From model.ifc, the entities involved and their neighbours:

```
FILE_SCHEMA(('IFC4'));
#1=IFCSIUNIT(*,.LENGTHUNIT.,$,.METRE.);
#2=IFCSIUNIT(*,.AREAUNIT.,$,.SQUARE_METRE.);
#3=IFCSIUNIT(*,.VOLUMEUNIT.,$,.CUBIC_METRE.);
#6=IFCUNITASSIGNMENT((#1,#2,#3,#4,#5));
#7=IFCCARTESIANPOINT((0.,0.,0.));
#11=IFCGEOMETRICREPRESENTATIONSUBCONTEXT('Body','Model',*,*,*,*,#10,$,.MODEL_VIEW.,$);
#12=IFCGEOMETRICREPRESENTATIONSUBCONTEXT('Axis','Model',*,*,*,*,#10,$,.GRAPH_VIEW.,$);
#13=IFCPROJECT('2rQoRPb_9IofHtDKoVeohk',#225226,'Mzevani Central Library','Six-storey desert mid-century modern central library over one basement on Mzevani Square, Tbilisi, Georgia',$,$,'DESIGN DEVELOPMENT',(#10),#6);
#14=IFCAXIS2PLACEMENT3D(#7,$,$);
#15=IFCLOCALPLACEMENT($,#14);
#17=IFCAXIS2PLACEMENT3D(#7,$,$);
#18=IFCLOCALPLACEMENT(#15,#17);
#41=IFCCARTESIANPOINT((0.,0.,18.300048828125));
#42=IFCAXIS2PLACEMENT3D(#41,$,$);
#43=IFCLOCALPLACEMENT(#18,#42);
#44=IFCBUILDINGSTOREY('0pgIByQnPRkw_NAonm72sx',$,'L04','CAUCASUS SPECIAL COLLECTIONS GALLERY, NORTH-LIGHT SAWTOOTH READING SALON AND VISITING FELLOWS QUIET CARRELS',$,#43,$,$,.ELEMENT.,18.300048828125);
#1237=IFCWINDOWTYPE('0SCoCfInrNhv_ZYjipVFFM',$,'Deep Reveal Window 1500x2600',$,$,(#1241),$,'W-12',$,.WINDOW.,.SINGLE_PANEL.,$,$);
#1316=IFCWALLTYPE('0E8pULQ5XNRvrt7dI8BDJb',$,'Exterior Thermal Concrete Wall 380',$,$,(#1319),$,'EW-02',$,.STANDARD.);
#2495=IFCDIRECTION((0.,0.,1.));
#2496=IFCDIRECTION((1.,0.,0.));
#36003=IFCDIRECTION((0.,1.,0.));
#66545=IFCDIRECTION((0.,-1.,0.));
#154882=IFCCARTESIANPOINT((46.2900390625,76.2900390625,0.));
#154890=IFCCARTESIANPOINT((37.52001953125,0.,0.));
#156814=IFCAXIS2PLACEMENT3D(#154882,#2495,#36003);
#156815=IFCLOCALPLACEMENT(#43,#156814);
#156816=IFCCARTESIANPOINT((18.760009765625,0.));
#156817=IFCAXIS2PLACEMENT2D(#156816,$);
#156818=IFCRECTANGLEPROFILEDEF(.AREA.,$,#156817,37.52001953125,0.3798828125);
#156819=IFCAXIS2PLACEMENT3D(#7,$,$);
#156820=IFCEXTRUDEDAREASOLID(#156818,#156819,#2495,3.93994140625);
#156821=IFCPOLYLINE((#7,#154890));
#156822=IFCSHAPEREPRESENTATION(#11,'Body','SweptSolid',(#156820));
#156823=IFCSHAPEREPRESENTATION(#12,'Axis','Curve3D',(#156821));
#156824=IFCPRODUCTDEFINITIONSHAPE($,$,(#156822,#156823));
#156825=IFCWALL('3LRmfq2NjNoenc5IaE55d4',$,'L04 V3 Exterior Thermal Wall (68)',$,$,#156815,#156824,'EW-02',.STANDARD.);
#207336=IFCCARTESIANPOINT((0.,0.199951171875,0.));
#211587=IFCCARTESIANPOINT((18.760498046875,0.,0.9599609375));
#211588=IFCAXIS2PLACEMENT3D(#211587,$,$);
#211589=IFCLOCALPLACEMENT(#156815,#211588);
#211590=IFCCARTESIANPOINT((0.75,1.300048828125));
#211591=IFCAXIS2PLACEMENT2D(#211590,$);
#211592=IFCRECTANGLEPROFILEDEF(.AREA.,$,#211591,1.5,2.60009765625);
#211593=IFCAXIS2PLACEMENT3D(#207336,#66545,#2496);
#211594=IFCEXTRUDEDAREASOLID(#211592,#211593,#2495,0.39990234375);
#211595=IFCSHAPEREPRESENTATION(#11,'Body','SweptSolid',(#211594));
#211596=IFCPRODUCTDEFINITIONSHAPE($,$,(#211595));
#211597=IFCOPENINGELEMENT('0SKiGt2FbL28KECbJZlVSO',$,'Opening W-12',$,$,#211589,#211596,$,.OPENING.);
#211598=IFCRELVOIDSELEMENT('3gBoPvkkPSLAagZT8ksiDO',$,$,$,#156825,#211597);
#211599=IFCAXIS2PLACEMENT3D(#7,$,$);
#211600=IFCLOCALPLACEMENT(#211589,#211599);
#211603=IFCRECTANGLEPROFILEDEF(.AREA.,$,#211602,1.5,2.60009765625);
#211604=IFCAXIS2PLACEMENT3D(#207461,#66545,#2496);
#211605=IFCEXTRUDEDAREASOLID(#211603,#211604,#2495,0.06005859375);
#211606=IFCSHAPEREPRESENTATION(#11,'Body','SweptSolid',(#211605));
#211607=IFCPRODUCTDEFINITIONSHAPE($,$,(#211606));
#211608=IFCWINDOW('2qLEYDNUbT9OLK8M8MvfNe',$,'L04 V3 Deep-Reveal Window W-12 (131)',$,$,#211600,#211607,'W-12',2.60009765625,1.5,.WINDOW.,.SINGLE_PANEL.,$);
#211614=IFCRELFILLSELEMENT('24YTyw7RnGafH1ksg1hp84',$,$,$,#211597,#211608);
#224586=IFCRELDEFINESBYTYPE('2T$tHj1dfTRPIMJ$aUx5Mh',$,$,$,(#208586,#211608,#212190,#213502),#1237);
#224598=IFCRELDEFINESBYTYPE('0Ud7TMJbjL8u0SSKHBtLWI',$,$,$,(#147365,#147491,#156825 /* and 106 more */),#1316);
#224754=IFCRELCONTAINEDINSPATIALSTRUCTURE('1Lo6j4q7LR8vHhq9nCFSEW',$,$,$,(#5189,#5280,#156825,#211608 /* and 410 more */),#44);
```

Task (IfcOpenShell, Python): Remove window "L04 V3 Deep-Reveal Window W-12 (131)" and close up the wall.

```python
import ifcopenshell
import ifcopenshell.api.feature
import ifcopenshell.api.root
import ifcopenshell.geom
import ifcopenshell.util.shape

model = ifcopenshell.open("model.ifc")
settings = ifcopenshell.geom.settings()


def volume(element):
    """Net volume in cubic metres, openings subtracted."""
    shape = ifcopenshell.geom.create_shape(settings, element)
    return ifcopenshell.util.shape.get_volume(shape.geometry)


window = model.by_id(211608)
opening = window.FillsVoids[0].RelatingOpeningElement
wall = opening.VoidsElements[0].RelatingBuildingElement
before = volume(wall)

ifcopenshell.api.root.remove_product(model, product=window)
ifcopenshell.api.feature.remove_feature(model, feature=opening)

after = volume(wall)

print(f"wall volume {before:.3f} -> {after:.3f} m3")

model.write("model_rev.ifc")
```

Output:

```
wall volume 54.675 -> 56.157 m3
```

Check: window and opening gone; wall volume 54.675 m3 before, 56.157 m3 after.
